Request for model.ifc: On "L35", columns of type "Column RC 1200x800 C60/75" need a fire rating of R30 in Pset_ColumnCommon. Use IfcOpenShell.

First a look at what the model holds.

```python
import ifcopenshell
import ifcopenshell.util.element

model = ifcopenshell.open("model.ifc")
print(model.schema)
storey = next(s for s in model.by_type("IfcBuildingStorey") if s.Name == "L35")
columns = [e for e in ifcopenshell.util.element.get_decomposition(storey) if e.is_a("IfcColumn")]
seen = {}
for e in columns:
    element_type = ifcopenshell.util.element.get_type(e)
    key = (element_type.Name if element_type != e and element_type else None, ifcopenshell.util.element.get_pset(e, "Pset_ColumnCommon", "FireRating"))
    seen[key] = seen.get(key, 0) + 1
for (name, value), count in sorted(seen.items(), key=str):
    print(count, "x", name, "|", value)
```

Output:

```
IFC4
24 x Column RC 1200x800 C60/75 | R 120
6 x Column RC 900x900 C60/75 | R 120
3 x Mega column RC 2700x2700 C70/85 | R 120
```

```python
import ifcopenshell
import ifcopenshell.api.pset
import ifcopenshell.util.element

model = ifcopenshell.open("model.ifc")

storey = next(s for s in model.by_type("IfcBuildingStorey") if s.Name == "L35")
columns = [e for e in ifcopenshell.util.element.get_decomposition(storey) if e.is_a("IfcColumn")]

count = 0
for e in columns:
    element_type = ifcopenshell.util.element.get_type(e)
    if element_type in (None, e) or element_type.Name != "Column RC 1200x800 C60/75":
        continue
    found = ifcopenshell.util.element.get_pset(e, "Pset_ColumnCommon", should_inherit=False)
    if found:
        pset = model.by_id(found["id"])
        if len(ifcopenshell.util.element.get_elements_by_pset(pset)) > 1:
            pset = ifcopenshell.api.pset.unshare_pset(model, products=[e], pset=pset)[0]
    else:
        pset = ifcopenshell.api.pset.add_pset(model, product=e, name="Pset_ColumnCommon")
    ifcopenshell.api.pset.edit_pset(model, pset=pset, properties={"FireRating": "R30"})
    count += 1

print(count, "columns updated")

model.write("model_edited.ifc")
```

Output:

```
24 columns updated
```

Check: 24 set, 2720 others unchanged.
